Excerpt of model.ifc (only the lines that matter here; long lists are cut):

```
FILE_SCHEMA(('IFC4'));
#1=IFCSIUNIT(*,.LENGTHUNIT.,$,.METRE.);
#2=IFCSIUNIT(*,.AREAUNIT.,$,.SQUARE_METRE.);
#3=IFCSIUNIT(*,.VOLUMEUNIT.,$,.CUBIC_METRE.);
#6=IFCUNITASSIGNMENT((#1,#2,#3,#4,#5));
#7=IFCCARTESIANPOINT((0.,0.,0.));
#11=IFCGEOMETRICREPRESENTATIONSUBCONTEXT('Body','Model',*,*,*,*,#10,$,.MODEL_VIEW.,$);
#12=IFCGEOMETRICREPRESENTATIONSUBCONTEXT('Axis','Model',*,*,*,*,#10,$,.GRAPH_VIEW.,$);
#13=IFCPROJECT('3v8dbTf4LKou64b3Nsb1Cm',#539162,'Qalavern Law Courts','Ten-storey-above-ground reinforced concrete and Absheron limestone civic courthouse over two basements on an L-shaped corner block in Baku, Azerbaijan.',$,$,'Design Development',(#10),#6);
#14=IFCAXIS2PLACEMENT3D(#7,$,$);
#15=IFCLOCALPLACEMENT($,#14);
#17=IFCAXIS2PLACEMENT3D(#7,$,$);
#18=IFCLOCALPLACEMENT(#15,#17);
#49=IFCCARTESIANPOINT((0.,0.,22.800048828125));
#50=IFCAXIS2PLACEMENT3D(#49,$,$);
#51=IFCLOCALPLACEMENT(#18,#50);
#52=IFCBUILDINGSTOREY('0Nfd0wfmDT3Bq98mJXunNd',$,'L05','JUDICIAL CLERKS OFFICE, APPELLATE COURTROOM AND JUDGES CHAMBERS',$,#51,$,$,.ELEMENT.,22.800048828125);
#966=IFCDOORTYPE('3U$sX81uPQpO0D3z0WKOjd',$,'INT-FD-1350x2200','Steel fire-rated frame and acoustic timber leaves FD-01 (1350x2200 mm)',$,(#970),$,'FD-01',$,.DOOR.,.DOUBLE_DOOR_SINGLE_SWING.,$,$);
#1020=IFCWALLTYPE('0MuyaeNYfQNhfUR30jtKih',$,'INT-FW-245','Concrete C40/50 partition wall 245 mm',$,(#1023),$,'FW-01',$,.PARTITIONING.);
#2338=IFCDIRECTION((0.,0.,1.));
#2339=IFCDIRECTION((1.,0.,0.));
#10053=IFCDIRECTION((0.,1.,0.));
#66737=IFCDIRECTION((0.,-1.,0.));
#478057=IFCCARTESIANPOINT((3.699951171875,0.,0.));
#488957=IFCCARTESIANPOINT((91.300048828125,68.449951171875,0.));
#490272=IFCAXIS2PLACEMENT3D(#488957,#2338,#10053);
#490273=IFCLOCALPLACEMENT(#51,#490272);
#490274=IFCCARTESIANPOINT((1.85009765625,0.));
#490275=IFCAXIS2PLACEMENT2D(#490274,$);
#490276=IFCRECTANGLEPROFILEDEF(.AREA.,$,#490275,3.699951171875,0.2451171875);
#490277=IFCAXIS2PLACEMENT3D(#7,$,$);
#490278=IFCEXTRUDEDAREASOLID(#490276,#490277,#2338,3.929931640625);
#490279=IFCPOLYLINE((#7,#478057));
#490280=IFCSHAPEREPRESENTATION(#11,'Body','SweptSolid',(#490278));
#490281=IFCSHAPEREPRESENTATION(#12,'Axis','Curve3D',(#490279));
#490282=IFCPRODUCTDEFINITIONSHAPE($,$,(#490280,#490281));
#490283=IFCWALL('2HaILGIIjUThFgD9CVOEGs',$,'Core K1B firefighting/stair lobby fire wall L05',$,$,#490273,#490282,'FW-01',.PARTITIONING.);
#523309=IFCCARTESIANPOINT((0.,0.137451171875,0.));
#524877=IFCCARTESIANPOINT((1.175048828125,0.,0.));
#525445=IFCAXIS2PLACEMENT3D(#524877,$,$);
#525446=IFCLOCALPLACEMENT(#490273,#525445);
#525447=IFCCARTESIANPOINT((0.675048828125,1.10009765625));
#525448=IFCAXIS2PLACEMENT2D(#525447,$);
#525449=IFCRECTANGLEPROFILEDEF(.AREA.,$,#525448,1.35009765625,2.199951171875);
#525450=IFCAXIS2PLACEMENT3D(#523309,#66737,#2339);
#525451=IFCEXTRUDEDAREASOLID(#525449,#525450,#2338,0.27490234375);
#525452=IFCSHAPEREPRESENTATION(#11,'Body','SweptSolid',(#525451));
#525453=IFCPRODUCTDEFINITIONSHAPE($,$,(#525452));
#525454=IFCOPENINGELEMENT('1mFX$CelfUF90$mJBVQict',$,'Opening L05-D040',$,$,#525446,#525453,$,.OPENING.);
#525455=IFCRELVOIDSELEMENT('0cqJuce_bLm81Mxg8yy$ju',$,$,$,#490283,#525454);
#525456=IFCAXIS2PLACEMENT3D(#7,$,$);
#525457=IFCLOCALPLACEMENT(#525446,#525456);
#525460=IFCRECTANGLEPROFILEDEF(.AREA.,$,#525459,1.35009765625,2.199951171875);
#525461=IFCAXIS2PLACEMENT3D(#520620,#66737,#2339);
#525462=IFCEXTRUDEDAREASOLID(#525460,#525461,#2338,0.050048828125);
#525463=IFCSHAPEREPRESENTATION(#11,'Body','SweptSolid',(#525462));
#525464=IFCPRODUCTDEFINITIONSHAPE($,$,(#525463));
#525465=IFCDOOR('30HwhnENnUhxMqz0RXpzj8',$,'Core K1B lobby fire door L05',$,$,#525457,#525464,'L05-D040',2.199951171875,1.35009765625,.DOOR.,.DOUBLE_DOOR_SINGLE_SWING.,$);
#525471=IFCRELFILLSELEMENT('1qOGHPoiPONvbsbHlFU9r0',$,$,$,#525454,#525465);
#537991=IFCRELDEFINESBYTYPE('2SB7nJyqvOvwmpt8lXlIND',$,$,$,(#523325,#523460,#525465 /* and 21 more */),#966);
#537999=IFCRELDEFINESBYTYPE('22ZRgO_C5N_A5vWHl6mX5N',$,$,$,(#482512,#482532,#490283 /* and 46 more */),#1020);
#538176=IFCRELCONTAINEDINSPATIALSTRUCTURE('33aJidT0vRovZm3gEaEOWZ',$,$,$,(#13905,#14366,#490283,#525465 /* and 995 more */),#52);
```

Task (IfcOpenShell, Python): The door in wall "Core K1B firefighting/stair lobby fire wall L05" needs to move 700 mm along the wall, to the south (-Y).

```python
import ifcopenshell
import ifcopenshell.api.geometry
import ifcopenshell.util.placement

model = ifcopenshell.open("model.ifc")

door = model.by_guid("30HwhnENnUhxMqz0RXpzj8")
opening = door.FillsVoids[0].RelatingOpeningElement
wall = opening.VoidsElements[0].RelatingBuildingElement

wall_matrix = ifcopenshell.util.placement.get_local_placement(wall.ObjectPlacement)
shift = wall_matrix[:3, 0] * -0.7
before = ifcopenshell.util.placement.get_local_placement(door.ObjectPlacement)[:3, 3].copy()

# The door is placed relative to its opening, so it follows when the opening moves.
matrix = ifcopenshell.util.placement.get_local_placement(opening.ObjectPlacement)
matrix[:3, 3] += shift
ifcopenshell.api.geometry.edit_object_placement(
    model, product=opening, matrix=matrix, is_si=False, should_transform_children=True
)

after = ifcopenshell.util.placement.get_local_placement(door.ObjectPlacement)[:3, 3]
print("door moved by", (after - before).round(3) + 0.0)

model.write("model-out.ifc")
```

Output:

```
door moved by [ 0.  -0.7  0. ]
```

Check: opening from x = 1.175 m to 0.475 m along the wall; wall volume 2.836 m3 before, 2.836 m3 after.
